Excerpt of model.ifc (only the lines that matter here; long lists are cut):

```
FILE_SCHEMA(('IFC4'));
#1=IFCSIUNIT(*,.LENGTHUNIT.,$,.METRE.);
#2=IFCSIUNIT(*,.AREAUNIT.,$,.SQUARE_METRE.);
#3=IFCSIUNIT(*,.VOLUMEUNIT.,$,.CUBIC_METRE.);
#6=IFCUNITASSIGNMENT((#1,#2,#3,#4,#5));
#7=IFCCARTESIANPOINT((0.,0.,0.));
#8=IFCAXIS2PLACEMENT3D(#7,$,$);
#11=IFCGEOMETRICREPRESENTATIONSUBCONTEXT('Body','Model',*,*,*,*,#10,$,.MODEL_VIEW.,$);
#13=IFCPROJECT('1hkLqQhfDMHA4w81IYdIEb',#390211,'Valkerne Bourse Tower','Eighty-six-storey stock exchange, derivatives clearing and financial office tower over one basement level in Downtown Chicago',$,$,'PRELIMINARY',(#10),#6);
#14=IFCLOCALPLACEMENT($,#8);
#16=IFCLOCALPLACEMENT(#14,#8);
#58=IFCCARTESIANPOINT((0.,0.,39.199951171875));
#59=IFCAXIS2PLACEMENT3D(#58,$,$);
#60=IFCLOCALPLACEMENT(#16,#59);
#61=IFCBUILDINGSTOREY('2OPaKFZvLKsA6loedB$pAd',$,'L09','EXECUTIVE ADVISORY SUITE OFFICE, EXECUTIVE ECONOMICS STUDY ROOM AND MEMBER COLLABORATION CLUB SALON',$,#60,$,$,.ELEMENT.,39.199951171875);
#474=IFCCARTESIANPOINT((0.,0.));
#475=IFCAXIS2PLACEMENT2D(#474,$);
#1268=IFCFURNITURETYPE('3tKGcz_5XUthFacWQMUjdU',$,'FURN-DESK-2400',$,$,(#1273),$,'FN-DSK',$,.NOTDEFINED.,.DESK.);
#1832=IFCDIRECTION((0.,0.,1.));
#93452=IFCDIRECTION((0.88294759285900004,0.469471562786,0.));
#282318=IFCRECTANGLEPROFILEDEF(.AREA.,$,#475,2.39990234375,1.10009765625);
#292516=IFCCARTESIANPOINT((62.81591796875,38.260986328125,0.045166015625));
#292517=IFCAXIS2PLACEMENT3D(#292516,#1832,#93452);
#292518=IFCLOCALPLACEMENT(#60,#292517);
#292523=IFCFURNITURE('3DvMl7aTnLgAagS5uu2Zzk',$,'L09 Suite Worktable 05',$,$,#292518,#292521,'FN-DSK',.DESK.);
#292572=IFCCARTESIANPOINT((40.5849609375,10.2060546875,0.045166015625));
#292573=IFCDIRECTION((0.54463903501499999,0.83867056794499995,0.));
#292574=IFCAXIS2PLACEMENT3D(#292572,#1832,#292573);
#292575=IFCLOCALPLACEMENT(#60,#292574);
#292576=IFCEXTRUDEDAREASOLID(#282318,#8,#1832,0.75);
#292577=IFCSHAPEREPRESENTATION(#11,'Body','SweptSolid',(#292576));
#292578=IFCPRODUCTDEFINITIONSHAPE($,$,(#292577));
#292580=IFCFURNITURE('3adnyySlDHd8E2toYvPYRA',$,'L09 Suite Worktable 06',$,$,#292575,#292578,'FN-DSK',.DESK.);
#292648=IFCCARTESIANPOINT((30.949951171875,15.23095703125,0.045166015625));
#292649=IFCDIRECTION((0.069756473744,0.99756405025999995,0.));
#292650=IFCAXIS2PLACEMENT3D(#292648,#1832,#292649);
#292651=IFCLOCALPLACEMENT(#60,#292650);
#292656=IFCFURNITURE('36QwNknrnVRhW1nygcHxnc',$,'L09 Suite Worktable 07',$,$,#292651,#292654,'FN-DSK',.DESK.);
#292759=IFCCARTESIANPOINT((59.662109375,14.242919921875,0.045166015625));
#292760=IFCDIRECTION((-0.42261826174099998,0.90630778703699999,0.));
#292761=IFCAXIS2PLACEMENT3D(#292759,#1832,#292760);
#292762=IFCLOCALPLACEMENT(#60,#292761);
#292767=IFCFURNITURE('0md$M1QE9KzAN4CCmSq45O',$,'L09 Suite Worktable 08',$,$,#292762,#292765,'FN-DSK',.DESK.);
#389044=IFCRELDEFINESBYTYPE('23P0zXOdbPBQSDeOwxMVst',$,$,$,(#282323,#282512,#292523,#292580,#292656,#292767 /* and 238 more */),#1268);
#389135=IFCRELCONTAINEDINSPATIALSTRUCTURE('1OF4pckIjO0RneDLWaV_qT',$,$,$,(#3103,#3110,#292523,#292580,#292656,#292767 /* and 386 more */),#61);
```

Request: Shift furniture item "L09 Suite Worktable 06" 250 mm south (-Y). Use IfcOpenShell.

```python
import ifcopenshell
import ifcopenshell.api.geometry
import ifcopenshell.util.placement
import ifcopenshell.util.unit

model = ifcopenshell.open("model.ifc")
unit_scale = ifcopenshell.util.unit.calculate_unit_scale(model)

item = model.by_guid("3adnyySlDHd8E2toYvPYRA")
matrix = ifcopenshell.util.placement.get_local_placement(item.ObjectPlacement)
matrix[1, 3] -= 0.25 / unit_scale
ifcopenshell.api.geometry.edit_object_placement(model, product=item, matrix=matrix, is_si=False)

print(ifcopenshell.util.placement.get_local_placement(item.ObjectPlacement).round(3) + 0.0)

model.write("model_rev.ifc")
```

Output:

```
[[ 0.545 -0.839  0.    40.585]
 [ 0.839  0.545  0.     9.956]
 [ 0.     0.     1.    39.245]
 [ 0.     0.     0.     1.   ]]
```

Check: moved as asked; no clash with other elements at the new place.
